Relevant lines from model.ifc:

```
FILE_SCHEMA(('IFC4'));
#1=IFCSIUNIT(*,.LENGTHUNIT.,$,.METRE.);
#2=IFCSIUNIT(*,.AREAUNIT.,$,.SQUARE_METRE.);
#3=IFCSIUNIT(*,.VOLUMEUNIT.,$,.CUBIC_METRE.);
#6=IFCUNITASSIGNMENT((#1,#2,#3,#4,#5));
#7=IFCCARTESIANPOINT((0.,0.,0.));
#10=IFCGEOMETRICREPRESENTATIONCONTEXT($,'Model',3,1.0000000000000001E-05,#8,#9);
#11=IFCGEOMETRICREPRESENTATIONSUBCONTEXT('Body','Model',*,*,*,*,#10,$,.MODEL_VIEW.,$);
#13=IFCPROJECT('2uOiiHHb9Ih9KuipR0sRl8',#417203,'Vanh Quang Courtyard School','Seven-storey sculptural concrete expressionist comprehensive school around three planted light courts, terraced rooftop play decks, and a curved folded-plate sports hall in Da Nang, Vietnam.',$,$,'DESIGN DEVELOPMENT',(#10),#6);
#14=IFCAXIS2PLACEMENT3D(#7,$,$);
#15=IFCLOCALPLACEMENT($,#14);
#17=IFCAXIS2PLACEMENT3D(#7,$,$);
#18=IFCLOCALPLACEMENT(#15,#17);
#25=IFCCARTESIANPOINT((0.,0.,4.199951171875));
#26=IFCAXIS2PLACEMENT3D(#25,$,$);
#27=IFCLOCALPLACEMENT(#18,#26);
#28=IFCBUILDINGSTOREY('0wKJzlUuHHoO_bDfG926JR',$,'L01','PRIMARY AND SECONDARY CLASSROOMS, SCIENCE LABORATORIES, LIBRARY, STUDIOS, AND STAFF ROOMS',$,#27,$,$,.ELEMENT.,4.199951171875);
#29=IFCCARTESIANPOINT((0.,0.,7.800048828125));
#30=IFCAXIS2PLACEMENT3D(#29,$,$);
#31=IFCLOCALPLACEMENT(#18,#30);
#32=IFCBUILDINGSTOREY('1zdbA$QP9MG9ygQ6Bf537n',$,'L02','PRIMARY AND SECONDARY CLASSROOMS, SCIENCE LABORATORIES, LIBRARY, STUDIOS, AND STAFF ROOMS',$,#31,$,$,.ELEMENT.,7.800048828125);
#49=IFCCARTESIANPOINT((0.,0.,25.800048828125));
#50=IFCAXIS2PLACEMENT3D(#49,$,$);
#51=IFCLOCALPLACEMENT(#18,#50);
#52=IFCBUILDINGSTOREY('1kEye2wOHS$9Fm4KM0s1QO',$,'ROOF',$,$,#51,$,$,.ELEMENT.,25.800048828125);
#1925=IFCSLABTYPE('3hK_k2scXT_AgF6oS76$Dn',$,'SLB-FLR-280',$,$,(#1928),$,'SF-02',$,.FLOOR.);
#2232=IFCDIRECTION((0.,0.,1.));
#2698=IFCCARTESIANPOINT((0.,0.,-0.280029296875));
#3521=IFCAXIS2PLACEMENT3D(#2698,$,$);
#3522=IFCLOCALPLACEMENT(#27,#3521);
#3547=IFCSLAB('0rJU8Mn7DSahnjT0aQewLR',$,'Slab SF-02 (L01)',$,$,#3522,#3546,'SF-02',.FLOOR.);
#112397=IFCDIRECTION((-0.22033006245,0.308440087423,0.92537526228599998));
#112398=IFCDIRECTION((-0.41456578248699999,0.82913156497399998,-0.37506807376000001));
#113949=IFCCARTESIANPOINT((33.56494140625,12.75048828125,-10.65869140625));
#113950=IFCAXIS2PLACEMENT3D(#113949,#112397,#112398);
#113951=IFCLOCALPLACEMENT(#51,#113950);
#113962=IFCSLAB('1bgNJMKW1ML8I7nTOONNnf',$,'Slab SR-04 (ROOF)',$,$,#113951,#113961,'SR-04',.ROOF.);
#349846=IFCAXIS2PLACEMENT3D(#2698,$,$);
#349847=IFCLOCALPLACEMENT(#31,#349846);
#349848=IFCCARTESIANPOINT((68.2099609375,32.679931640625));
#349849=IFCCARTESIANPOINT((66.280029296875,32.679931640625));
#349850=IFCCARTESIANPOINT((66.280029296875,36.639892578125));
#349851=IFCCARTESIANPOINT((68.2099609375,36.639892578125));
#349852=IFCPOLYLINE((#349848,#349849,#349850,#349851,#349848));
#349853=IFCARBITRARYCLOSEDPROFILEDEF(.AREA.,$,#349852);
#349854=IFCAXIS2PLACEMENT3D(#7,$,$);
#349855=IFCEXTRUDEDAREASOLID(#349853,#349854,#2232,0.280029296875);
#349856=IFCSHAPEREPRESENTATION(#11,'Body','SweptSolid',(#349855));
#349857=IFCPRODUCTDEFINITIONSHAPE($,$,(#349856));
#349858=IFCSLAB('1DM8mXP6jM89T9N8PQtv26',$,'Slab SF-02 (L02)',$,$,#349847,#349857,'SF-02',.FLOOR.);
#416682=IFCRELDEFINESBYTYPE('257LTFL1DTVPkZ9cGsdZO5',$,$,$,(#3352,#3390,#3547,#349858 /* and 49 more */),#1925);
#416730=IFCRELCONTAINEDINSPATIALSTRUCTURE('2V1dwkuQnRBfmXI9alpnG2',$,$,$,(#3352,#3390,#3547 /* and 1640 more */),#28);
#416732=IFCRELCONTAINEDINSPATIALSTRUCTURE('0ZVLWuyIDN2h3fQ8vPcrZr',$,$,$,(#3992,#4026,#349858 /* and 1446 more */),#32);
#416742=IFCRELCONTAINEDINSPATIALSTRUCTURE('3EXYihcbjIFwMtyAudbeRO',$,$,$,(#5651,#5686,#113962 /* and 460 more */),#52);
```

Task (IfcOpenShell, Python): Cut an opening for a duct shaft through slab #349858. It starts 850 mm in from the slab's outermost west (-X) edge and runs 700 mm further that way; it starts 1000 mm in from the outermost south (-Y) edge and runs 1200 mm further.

```python
import numpy as np
import ifcopenshell
import ifcopenshell.api.feature
import ifcopenshell.api.geometry
import ifcopenshell.api.root
import ifcopenshell.geom
import ifcopenshell.util.placement
import ifcopenshell.util.representation
import ifcopenshell.util.shape
import ifcopenshell.util.unit

model = ifcopenshell.open("model.ifc")
unit_scale = ifcopenshell.util.unit.calculate_unit_scale(model)
settings = ifcopenshell.geom.settings()


def volume(element):
    """Net volume in cubic metres, openings subtracted."""
    shape = ifcopenshell.geom.create_shape(settings, element)
    return ifcopenshell.util.shape.get_volume(shape.geometry)


slab = model.by_guid("1DM8mXP6jM89T9N8PQtv26")
before = volume(slab)

# Extent in the slab's own axes, in metres. The edges named are its -X and -Y sides.
slab_shape = ifcopenshell.geom.create_shape(settings, slab)
vertices = ifcopenshell.util.shape.get_vertices(slab_shape.geometry)
x_min, y_min, bottom = vertices.min(axis=0)
top = vertices[:, 2].max()

opening = ifcopenshell.api.root.create_entity(model, ifc_class="IfcOpeningElement", name="Duct shaft opening", predefined_type="OPENING")
context = ifcopenshell.util.representation.get_context(model, "Model", "Body", "MODEL_VIEW")
width, depth = 0.7, 1.2
outline = [(0.0, 0.0), (width, 0.0), (width, depth), (0.0, depth), (0.0, 0.0)]
# Overshoot both faces by 50 mm so the cut is clean.
shape = ifcopenshell.api.geometry.add_slab_representation(
    model, context=context, depth=top - bottom + 0.1, polyline=outline
)
ifcopenshell.api.geometry.assign_representation(model, product=opening, representation=shape)

matrix = ifcopenshell.util.placement.get_local_placement(slab.ObjectPlacement)
matrix[:, 3] = matrix @ np.append(np.array([x_min + 0.85, y_min + 1, bottom - 0.05]) / unit_scale, 1.0)
ifcopenshell.api.geometry.edit_object_placement(model, product=opening, matrix=matrix, is_si=False)
ifcopenshell.api.feature.add_feature(model, feature=opening, element=slab)

after = volume(slab)

print(f"slab volume {before:.3f} -> {after:.3f} m3")

model.write("model-out.ifc")
```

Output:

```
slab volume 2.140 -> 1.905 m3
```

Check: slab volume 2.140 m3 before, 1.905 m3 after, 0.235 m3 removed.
